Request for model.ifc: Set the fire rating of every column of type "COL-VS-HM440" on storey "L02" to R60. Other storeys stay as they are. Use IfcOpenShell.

First a look at what the model holds.

```python
import ifcopenshell
import ifcopenshell.util.element

model = ifcopenshell.open("model.ifc")
print(model.schema)
storey = next(s for s in model.by_type("IfcBuildingStorey") if s.Name == "L02")
columns = [e for e in ifcopenshell.util.element.get_decomposition(storey) if e.is_a("IfcColumn")]
seen = {}
for e in columns:
    element_type = ifcopenshell.util.element.get_type(e)
    key = (element_type.Name if element_type != e and element_type else None, ifcopenshell.util.element.get_pset(e, "Pset_ColumnCommon", "FireRating"))
    seen[key] = seen.get(key, 0) + 1
for (name, value), count in sorted(seen.items(), key=str):
    print(count, "x", name, "|", value)
```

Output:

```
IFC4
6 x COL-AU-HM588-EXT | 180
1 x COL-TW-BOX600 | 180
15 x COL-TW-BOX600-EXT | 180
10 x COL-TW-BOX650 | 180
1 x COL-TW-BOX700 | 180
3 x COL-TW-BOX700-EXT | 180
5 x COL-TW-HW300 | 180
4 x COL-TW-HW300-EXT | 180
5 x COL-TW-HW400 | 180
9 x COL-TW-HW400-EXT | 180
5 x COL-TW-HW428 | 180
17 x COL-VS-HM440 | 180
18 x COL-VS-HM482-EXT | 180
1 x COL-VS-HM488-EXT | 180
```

```python
import ifcopenshell
import ifcopenshell.api.pset
import ifcopenshell.util.element

model = ifcopenshell.open("model.ifc")

storey = next(s for s in model.by_type("IfcBuildingStorey") if s.Name == "L02")
columns = [e for e in ifcopenshell.util.element.get_decomposition(storey) if e.is_a("IfcColumn")]

count = 0
for e in columns:
    element_type = ifcopenshell.util.element.get_type(e)
    if element_type in (None, e) or element_type.Name != "COL-VS-HM440":
        continue
    # add_pset returns the element's existing set when there is one.
    pset = ifcopenshell.api.pset.add_pset(model, product=e, name="Pset_ColumnCommon")
    ifcopenshell.api.pset.edit_pset(model, pset=pset, properties={"FireRating": "R60"})
    count += 1

print(count, "columns updated")

model.write("model_updated.ifc")
```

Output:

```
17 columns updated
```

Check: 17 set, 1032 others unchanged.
